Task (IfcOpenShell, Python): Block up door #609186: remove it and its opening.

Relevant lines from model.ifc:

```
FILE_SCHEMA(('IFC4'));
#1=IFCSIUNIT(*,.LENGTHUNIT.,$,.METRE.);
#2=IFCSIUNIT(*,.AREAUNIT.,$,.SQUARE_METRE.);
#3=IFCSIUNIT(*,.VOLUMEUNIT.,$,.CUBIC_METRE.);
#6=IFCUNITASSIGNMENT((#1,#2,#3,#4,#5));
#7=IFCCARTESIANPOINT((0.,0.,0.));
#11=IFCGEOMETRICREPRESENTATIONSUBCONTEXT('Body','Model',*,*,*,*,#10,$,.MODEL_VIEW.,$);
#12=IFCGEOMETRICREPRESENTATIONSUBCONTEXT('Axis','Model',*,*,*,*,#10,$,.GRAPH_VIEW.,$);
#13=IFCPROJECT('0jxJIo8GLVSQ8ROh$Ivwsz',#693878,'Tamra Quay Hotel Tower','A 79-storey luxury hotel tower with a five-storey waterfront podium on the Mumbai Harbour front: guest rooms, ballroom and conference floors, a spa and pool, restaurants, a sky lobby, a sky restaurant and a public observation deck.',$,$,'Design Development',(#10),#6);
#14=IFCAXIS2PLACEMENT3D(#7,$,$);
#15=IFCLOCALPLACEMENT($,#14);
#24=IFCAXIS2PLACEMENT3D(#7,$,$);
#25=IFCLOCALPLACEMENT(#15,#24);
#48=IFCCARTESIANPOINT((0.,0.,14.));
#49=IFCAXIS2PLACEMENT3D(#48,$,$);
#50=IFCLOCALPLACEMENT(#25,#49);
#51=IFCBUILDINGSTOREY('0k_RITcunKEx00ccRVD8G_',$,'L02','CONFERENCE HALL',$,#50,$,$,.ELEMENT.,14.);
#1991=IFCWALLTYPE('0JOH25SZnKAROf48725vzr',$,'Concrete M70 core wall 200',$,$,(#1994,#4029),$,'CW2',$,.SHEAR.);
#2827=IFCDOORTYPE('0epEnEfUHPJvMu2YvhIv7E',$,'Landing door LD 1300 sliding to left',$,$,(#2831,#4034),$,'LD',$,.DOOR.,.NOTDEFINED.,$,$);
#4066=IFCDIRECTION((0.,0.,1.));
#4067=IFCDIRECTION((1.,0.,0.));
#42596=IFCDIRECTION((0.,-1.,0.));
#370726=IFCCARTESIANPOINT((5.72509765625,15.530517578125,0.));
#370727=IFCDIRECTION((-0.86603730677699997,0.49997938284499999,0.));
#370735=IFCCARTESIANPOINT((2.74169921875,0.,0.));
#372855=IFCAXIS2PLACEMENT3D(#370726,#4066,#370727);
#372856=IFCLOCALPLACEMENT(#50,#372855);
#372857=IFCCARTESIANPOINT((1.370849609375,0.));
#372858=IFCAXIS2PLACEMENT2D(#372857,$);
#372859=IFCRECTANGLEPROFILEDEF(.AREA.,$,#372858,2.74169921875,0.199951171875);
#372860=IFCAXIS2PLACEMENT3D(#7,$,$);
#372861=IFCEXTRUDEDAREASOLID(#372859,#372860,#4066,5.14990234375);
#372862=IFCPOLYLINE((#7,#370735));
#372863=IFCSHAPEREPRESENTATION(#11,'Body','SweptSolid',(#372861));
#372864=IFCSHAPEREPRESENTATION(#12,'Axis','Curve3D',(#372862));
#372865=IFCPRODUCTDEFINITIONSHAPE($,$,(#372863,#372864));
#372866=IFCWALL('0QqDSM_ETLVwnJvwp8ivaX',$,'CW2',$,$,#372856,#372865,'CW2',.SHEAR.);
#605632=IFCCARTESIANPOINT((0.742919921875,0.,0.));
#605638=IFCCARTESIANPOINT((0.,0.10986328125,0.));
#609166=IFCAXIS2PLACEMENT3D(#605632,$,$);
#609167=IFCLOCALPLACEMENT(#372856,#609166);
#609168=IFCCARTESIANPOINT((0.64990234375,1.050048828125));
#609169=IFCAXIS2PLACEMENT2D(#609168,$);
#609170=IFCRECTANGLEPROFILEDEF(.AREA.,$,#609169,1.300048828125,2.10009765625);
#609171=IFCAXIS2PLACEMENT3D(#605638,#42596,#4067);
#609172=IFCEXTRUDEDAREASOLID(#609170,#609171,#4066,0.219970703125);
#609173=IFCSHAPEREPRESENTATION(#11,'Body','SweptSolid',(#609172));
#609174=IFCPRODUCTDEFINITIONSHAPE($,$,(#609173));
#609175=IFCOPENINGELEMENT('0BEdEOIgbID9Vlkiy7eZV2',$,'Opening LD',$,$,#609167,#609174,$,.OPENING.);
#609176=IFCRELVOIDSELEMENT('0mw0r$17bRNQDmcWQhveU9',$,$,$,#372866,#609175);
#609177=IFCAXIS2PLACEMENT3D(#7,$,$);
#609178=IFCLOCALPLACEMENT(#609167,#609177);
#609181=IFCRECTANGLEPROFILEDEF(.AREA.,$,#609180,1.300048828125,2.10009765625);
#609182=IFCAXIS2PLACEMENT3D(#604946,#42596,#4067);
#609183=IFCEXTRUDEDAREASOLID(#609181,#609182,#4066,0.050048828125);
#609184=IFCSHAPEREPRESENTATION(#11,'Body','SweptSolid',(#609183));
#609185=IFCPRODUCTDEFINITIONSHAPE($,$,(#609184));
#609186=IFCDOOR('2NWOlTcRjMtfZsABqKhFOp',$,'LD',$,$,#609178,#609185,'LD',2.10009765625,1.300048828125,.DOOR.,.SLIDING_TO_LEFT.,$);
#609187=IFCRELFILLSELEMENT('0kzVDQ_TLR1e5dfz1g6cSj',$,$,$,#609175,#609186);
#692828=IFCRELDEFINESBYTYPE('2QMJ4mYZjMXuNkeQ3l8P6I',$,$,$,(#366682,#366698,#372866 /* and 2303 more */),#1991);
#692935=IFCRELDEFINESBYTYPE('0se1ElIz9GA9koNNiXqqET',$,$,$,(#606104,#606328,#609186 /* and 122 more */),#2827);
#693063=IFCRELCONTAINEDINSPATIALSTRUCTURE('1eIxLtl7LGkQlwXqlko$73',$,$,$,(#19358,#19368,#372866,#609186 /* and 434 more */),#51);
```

```python
import ifcopenshell
import ifcopenshell.api.feature
import ifcopenshell.api.root
import ifcopenshell.geom
import ifcopenshell.util.shape

model = ifcopenshell.open("model.ifc")
settings = ifcopenshell.geom.settings()


def volume(element):
    """Net volume in cubic metres, openings subtracted."""
    shape = ifcopenshell.geom.create_shape(settings, element)
    return ifcopenshell.util.shape.get_volume(shape.geometry)


door = model.by_guid("2NWOlTcRjMtfZsABqKhFOp")
opening = door.FillsVoids[0].RelatingOpeningElement
wall = opening.VoidsElements[0].RelatingBuildingElement
before = volume(wall)

ifcopenshell.api.root.remove_product(model, product=door)
ifcopenshell.api.feature.remove_feature(model, feature=opening)

after = volume(wall)

print(f"wall volume {before:.3f} -> {after:.3f} m3")

model.write("model-out.ifc")
```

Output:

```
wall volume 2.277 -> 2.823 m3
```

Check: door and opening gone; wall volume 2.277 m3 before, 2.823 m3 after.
